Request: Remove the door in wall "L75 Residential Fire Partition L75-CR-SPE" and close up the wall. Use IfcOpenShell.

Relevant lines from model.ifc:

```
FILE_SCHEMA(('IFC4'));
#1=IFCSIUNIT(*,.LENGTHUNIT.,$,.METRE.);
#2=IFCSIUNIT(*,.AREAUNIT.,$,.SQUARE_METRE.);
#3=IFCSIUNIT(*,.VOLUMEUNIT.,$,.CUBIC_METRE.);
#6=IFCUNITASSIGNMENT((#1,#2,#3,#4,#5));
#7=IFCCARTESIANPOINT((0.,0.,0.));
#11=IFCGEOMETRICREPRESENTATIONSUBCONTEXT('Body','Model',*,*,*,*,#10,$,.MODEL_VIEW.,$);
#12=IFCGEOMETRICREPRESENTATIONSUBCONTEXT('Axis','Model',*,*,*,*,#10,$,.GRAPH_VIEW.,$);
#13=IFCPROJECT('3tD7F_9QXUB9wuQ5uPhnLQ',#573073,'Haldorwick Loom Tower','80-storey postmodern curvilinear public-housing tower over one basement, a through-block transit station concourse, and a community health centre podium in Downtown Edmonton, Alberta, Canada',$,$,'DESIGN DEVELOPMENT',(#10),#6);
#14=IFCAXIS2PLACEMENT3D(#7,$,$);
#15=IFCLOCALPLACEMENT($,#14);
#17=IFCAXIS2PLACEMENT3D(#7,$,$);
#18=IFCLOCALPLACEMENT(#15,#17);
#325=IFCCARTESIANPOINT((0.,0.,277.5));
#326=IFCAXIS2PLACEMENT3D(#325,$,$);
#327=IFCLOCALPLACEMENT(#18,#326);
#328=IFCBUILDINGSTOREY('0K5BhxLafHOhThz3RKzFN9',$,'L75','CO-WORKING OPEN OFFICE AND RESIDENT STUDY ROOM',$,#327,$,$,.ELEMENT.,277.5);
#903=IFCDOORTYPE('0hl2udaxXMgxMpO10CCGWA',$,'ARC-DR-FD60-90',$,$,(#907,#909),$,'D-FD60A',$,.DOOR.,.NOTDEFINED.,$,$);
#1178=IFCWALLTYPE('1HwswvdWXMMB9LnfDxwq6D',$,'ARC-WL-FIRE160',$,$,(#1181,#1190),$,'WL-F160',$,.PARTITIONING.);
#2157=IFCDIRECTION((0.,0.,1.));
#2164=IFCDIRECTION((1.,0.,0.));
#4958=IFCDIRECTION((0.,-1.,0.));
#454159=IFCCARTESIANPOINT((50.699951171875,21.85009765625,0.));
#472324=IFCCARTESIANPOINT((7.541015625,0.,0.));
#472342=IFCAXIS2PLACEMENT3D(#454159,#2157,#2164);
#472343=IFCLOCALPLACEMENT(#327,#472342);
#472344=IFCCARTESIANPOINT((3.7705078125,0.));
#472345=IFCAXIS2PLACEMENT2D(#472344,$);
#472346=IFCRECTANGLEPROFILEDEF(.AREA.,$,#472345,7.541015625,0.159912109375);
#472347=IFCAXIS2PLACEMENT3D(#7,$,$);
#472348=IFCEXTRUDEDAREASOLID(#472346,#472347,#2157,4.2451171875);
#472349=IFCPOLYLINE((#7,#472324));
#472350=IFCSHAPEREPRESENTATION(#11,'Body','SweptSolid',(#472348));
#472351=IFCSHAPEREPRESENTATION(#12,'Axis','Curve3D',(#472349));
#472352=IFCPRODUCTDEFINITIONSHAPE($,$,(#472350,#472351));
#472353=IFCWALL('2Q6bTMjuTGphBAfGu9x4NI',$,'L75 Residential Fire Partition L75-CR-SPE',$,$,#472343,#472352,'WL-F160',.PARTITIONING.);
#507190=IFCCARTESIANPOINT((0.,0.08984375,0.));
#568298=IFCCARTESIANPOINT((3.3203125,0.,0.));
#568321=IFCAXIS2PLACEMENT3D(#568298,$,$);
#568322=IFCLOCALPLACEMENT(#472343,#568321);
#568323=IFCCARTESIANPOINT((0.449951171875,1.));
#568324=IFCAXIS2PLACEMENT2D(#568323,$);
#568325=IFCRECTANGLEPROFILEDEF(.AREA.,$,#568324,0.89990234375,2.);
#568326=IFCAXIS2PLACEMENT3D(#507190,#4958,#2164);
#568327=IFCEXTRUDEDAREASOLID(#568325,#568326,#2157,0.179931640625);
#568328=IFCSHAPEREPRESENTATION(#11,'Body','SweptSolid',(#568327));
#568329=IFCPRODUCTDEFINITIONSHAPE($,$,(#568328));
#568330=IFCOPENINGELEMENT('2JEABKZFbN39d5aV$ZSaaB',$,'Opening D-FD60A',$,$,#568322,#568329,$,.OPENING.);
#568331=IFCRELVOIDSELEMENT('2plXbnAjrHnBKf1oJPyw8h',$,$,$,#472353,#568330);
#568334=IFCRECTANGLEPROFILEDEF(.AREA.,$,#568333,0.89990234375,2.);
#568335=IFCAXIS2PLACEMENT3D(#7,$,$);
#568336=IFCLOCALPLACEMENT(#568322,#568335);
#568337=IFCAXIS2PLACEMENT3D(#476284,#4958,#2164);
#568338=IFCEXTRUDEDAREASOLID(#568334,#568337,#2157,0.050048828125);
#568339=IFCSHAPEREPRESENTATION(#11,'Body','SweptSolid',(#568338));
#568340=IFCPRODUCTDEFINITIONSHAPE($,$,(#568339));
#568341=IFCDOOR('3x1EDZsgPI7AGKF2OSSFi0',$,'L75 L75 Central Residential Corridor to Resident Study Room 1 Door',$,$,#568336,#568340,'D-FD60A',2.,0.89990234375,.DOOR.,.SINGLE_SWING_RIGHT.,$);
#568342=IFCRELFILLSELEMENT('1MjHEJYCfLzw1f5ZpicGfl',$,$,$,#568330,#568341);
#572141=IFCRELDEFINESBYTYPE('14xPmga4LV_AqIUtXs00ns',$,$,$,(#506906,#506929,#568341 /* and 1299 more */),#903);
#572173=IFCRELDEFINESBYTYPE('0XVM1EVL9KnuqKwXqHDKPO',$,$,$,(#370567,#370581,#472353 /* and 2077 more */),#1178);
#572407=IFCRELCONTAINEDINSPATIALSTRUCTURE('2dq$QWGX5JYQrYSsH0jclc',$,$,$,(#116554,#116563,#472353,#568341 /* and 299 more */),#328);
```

```python
import ifcopenshell
import ifcopenshell.api.feature
import ifcopenshell.api.root
import ifcopenshell.geom
import ifcopenshell.util.shape

model = ifcopenshell.open("model.ifc")
settings = ifcopenshell.geom.settings()


def volume(element):
    """Net volume in cubic metres, openings subtracted."""
    shape = ifcopenshell.geom.create_shape(settings, element)
    return ifcopenshell.util.shape.get_volume(shape.geometry)


door = model.by_id(568341)
opening = door.FillsVoids[0].RelatingOpeningElement
wall = opening.VoidsElements[0].RelatingBuildingElement
before = volume(wall)

ifcopenshell.api.root.remove_product(model, product=door)
ifcopenshell.api.feature.remove_feature(model, feature=opening)

after = volume(wall)

print(f"wall volume {before:.3f} -> {after:.3f} m3")

model.write("model-out.ifc")
```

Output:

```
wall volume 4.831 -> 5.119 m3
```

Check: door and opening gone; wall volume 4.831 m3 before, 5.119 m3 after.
